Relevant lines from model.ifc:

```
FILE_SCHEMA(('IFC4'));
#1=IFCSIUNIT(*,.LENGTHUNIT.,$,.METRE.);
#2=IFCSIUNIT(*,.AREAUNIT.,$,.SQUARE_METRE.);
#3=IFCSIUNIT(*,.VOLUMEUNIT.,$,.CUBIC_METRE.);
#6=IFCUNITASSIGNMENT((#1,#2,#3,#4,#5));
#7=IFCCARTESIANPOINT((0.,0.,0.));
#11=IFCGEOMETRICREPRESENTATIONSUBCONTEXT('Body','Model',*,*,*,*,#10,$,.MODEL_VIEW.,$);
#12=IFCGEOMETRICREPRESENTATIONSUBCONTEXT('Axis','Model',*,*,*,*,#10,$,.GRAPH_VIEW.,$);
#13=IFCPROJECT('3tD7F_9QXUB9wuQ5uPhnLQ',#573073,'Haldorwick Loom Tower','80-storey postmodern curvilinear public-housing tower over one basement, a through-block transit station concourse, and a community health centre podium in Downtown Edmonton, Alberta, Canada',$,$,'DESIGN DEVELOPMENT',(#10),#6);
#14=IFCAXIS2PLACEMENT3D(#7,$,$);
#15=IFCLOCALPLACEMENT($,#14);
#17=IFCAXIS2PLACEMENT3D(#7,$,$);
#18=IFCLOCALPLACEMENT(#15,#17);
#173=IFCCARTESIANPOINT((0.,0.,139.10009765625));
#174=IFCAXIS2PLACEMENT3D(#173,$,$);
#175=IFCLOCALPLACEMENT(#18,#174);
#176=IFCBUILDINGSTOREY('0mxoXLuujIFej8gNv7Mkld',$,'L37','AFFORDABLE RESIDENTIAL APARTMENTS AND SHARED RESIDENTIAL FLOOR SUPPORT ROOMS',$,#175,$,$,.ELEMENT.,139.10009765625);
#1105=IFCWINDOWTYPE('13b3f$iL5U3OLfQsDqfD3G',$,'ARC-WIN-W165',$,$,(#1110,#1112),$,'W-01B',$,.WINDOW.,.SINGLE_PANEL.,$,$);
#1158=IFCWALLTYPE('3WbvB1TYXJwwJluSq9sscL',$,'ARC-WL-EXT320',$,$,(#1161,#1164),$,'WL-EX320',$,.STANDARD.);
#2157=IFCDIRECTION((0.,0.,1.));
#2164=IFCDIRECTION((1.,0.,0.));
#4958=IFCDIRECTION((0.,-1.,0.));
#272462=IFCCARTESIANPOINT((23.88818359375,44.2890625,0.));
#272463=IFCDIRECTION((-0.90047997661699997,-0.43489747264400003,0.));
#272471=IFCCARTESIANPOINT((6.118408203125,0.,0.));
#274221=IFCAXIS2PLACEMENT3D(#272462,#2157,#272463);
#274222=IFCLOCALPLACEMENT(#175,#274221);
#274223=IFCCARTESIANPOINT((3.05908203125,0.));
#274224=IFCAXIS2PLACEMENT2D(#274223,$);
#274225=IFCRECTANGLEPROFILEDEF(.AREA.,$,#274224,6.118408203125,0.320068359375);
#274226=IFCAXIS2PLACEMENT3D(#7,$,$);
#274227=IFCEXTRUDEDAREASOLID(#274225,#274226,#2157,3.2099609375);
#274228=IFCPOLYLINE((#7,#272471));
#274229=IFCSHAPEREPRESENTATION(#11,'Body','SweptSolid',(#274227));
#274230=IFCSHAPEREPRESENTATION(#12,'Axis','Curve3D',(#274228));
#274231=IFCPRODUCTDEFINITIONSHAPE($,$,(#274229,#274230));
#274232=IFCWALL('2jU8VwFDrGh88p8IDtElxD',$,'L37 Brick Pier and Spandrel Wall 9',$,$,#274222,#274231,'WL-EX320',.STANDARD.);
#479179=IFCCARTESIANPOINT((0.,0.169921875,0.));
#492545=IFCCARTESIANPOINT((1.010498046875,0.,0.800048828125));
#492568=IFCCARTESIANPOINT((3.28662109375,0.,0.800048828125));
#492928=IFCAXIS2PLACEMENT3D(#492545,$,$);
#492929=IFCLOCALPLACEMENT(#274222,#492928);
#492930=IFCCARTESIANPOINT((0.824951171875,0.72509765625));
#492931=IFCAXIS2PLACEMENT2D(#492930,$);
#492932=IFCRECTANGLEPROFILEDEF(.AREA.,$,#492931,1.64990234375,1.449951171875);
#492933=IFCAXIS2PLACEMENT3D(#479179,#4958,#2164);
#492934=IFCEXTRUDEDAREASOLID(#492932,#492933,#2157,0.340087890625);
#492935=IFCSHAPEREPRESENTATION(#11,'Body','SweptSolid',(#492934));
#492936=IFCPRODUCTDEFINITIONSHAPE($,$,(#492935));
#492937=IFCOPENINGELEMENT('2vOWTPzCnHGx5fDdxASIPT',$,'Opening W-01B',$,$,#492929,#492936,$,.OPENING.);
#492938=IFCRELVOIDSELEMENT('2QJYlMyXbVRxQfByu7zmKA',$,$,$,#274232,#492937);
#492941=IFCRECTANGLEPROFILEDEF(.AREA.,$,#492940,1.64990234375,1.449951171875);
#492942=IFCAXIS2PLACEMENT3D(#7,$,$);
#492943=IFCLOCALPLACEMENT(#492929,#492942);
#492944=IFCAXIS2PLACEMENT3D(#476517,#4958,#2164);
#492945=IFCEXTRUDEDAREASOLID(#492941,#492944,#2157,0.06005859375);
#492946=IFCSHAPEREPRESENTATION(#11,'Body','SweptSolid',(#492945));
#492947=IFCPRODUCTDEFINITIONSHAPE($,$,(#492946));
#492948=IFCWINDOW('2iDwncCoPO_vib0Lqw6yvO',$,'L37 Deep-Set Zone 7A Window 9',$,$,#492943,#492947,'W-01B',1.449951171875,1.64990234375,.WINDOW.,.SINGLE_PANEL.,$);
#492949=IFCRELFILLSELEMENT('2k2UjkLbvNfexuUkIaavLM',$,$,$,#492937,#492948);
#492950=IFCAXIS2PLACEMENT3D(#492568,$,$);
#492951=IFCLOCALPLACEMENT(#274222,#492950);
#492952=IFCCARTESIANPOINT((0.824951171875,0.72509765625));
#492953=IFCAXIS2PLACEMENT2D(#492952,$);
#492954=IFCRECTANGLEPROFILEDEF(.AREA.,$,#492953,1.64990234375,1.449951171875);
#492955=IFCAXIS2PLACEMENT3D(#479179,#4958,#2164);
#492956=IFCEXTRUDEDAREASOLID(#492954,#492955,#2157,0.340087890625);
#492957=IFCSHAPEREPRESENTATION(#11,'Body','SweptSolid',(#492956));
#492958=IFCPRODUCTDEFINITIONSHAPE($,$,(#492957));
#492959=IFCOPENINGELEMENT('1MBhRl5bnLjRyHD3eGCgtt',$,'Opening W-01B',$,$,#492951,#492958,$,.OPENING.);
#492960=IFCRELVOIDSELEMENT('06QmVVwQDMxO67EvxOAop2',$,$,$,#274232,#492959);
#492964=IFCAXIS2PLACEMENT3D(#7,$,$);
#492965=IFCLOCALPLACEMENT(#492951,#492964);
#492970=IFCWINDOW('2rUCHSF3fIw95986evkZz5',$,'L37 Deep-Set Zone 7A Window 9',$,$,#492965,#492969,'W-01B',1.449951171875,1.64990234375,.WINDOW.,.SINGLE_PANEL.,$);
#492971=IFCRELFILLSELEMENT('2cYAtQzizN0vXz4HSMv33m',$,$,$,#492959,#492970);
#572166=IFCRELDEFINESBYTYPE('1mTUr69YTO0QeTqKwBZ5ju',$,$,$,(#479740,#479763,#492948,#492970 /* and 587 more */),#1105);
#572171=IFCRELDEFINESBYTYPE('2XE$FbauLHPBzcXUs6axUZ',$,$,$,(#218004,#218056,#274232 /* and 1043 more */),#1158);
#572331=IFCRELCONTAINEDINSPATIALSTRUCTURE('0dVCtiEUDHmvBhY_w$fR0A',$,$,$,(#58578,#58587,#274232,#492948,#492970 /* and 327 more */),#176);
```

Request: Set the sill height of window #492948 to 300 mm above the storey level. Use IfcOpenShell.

```python
import numpy as np
import ifcopenshell
import ifcopenshell.api.geometry
import ifcopenshell.geom
import ifcopenshell.util.element
import ifcopenshell.util.placement
import ifcopenshell.util.shape
import ifcopenshell.util.unit

model = ifcopenshell.open("model.ifc")
unit_scale = ifcopenshell.util.unit.calculate_unit_scale(model)

window = model.by_guid("2iDwncCoPO_vib0Lqw6yvO")
opening = window.FillsVoids[0].RelatingOpeningElement
storey = ifcopenshell.util.element.get_container(window, ifc_class="IfcBuildingStorey")
level = ifcopenshell.util.placement.get_local_placement(storey.ObjectPlacement)[2, 3]

# The opening's origin need not be at the sill, so measure its lowest point.
shape = ifcopenshell.geom.create_shape(ifcopenshell.geom.settings(), opening)
bottom = ifcopenshell.util.shape.get_shape_bottom_elevation(shape, shape.geometry) / unit_scale
dz = level + 0.3 - bottom

shift = np.array([0.0, 0.0, dz])
# The window is placed relative to its opening, so it follows when the opening moves.
matrix = ifcopenshell.util.placement.get_local_placement(opening.ObjectPlacement)
matrix[:3, 3] += shift
ifcopenshell.api.geometry.edit_object_placement(
    model, product=opening, matrix=matrix, is_si=False, should_transform_children=True
)

print(f"moved by {dz * unit_scale:+.3f} m")

model.write("model_edited.ifc")
```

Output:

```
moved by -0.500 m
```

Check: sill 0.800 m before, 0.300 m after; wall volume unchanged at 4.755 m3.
